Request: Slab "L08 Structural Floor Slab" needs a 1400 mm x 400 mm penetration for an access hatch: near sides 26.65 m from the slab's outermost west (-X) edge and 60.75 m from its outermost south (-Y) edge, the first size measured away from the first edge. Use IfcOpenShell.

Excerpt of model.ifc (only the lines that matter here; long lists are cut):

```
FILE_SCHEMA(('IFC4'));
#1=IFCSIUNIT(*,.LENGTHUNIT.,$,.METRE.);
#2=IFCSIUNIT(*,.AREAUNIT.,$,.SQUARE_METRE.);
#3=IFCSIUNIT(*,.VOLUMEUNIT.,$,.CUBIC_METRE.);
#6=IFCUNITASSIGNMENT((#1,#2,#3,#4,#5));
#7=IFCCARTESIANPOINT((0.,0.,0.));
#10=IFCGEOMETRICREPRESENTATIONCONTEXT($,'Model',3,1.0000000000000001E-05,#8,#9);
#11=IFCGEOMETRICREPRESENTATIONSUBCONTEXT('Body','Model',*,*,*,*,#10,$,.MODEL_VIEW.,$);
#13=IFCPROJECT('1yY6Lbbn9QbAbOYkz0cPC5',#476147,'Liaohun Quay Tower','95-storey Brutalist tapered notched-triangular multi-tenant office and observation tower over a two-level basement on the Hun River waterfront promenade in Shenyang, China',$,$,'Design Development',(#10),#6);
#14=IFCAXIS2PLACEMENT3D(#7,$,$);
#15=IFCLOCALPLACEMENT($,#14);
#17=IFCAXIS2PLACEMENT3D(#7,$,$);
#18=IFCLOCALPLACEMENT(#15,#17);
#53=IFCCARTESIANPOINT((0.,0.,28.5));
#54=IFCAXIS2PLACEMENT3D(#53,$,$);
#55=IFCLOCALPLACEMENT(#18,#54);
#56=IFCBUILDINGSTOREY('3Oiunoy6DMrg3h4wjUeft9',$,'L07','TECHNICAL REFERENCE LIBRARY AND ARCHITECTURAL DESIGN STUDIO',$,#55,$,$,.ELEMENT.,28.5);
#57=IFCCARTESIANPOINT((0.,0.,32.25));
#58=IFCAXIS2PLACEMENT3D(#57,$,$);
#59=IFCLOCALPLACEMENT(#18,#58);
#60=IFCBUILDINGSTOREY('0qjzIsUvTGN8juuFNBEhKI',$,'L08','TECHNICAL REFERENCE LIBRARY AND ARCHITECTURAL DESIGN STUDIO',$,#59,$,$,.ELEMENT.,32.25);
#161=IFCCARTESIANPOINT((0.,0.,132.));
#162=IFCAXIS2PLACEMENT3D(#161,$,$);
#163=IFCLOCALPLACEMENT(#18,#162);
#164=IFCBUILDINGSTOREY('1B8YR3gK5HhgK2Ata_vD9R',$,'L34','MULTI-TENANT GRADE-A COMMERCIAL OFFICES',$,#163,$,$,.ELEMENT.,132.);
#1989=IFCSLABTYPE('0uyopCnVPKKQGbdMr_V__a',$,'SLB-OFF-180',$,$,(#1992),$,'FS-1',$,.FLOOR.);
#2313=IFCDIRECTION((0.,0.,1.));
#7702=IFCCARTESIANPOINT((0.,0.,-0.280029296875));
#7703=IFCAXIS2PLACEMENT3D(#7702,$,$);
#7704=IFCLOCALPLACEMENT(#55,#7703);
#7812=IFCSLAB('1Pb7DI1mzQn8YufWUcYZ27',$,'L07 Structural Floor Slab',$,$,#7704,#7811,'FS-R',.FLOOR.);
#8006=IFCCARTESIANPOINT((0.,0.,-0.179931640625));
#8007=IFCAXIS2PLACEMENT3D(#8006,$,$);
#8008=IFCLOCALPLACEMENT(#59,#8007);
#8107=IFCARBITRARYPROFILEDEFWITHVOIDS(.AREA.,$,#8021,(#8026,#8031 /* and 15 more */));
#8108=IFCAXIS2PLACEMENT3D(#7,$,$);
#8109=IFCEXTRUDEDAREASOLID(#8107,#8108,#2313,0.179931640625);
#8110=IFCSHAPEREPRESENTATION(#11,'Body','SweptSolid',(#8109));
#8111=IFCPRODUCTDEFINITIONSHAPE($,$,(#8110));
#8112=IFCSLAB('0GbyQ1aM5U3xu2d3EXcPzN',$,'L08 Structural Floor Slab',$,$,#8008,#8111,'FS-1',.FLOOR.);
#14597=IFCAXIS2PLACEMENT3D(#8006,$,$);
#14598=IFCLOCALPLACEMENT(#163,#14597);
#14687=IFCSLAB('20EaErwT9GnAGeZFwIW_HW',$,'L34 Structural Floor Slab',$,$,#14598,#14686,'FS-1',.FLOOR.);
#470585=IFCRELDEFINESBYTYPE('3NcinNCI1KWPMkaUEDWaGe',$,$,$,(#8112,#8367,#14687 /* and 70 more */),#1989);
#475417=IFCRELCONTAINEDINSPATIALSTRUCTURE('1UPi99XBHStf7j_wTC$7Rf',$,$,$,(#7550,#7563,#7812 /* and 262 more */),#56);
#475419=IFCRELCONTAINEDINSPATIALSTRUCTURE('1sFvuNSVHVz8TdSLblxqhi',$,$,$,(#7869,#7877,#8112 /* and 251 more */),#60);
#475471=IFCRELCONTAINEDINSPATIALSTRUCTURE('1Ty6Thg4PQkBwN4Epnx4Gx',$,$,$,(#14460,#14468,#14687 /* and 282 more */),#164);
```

```python
import numpy as np
import ifcopenshell
import ifcopenshell.api.feature
import ifcopenshell.api.geometry
import ifcopenshell.api.root
import ifcopenshell.geom
import ifcopenshell.util.placement
import ifcopenshell.util.representation
import ifcopenshell.util.shape
import ifcopenshell.util.unit

model = ifcopenshell.open("model.ifc")
unit_scale = ifcopenshell.util.unit.calculate_unit_scale(model)
settings = ifcopenshell.geom.settings()


def volume(element):
    """Net volume in cubic metres, openings subtracted."""
    shape = ifcopenshell.geom.create_shape(settings, element)
    return ifcopenshell.util.shape.get_volume(shape.geometry)


slab = model.by_guid("0GbyQ1aM5U3xu2d3EXcPzN")
before = volume(slab)

# Extent in the slab's own axes, in metres. The edges named are its -X and -Y sides.
slab_shape = ifcopenshell.geom.create_shape(settings, slab)
vertices = ifcopenshell.util.shape.get_vertices(slab_shape.geometry)
x_min, y_min, bottom = vertices.min(axis=0)
top = vertices[:, 2].max()

opening = ifcopenshell.api.root.create_entity(model, ifc_class="IfcOpeningElement", name="Access hatch opening", predefined_type="OPENING")
context = ifcopenshell.util.representation.get_context(model, "Model", "Body", "MODEL_VIEW")
width, depth = 1.4, 0.4
outline = [(0.0, 0.0), (width, 0.0), (width, depth), (0.0, depth), (0.0, 0.0)]
# Overshoot both faces by 50 mm so the cut is clean.
shape = ifcopenshell.api.geometry.add_slab_representation(
    model, context=context, depth=top - bottom + 0.1, polyline=outline
)
ifcopenshell.api.geometry.assign_representation(model, product=opening, representation=shape)

matrix = ifcopenshell.util.placement.get_local_placement(slab.ObjectPlacement)
matrix[:, 3] = matrix @ np.append(np.array([x_min + 26.65, y_min + 60.75, bottom - 0.05]) / unit_scale, 1.0)
ifcopenshell.api.geometry.edit_object_placement(model, product=opening, matrix=matrix, is_si=False)
ifcopenshell.api.feature.add_feature(model, feature=opening, element=slab)

after = volume(slab)

print(f"slab volume {before:.3f} -> {after:.3f} m3")

model.write("model_updated.ifc")
```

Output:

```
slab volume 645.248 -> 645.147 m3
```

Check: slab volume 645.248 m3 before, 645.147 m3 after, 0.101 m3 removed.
